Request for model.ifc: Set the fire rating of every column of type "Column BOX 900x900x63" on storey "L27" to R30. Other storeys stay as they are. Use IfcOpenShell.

First a look at what the model holds.

```python
import ifcopenshell
import ifcopenshell.util.element

model = ifcopenshell.open("model.ifc")
print(model.schema)
storey = next(s for s in model.by_type("IfcBuildingStorey") if s.Name == "L27")
columns = [e for e in ifcopenshell.util.element.get_decomposition(storey) if e.is_a("IfcColumn")]
seen = {}
for e in columns:
    element_type = ifcopenshell.util.element.get_type(e)
    key = (element_type.Name if element_type != e and element_type else None, ifcopenshell.util.element.get_pset(e, "Pset_ColumnCommon", "FireRating"))
    seen[key] = seen.get(key, 0) + 1
for (name, value), count in sorted(seen.items(), key=str):
    print(count, "x", name, "|", value)
```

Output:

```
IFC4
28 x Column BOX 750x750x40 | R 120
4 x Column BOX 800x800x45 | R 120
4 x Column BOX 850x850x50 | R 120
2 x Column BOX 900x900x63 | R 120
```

```python
import ifcopenshell
import ifcopenshell.api.pset
import ifcopenshell.util.element

model = ifcopenshell.open("model.ifc")

storey = next(s for s in model.by_type("IfcBuildingStorey") if s.Name == "L27")
columns = [e for e in ifcopenshell.util.element.get_decomposition(storey) if e.is_a("IfcColumn")]

count = 0
for e in columns:
    element_type = ifcopenshell.util.element.get_type(e)
    if element_type in (None, e) or element_type.Name != "Column BOX 900x900x63":
        continue
    found = ifcopenshell.util.element.get_pset(e, "Pset_ColumnCommon", should_inherit=False)
    if found:
        pset = model.by_id(found["id"])
        if len(ifcopenshell.util.element.get_elements_by_pset(pset)) > 1:
            pset = ifcopenshell.api.pset.unshare_pset(model, products=[e], pset=pset)[0]
    else:
        pset = ifcopenshell.api.pset.add_pset(model, product=e, name="Pset_ColumnCommon")
    ifcopenshell.api.pset.edit_pset(model, pset=pset, properties={"FireRating": "R30"})
    count += 1

print(count, "columns updated")

model.write("model_edited.ifc")
```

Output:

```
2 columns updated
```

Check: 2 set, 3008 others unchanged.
